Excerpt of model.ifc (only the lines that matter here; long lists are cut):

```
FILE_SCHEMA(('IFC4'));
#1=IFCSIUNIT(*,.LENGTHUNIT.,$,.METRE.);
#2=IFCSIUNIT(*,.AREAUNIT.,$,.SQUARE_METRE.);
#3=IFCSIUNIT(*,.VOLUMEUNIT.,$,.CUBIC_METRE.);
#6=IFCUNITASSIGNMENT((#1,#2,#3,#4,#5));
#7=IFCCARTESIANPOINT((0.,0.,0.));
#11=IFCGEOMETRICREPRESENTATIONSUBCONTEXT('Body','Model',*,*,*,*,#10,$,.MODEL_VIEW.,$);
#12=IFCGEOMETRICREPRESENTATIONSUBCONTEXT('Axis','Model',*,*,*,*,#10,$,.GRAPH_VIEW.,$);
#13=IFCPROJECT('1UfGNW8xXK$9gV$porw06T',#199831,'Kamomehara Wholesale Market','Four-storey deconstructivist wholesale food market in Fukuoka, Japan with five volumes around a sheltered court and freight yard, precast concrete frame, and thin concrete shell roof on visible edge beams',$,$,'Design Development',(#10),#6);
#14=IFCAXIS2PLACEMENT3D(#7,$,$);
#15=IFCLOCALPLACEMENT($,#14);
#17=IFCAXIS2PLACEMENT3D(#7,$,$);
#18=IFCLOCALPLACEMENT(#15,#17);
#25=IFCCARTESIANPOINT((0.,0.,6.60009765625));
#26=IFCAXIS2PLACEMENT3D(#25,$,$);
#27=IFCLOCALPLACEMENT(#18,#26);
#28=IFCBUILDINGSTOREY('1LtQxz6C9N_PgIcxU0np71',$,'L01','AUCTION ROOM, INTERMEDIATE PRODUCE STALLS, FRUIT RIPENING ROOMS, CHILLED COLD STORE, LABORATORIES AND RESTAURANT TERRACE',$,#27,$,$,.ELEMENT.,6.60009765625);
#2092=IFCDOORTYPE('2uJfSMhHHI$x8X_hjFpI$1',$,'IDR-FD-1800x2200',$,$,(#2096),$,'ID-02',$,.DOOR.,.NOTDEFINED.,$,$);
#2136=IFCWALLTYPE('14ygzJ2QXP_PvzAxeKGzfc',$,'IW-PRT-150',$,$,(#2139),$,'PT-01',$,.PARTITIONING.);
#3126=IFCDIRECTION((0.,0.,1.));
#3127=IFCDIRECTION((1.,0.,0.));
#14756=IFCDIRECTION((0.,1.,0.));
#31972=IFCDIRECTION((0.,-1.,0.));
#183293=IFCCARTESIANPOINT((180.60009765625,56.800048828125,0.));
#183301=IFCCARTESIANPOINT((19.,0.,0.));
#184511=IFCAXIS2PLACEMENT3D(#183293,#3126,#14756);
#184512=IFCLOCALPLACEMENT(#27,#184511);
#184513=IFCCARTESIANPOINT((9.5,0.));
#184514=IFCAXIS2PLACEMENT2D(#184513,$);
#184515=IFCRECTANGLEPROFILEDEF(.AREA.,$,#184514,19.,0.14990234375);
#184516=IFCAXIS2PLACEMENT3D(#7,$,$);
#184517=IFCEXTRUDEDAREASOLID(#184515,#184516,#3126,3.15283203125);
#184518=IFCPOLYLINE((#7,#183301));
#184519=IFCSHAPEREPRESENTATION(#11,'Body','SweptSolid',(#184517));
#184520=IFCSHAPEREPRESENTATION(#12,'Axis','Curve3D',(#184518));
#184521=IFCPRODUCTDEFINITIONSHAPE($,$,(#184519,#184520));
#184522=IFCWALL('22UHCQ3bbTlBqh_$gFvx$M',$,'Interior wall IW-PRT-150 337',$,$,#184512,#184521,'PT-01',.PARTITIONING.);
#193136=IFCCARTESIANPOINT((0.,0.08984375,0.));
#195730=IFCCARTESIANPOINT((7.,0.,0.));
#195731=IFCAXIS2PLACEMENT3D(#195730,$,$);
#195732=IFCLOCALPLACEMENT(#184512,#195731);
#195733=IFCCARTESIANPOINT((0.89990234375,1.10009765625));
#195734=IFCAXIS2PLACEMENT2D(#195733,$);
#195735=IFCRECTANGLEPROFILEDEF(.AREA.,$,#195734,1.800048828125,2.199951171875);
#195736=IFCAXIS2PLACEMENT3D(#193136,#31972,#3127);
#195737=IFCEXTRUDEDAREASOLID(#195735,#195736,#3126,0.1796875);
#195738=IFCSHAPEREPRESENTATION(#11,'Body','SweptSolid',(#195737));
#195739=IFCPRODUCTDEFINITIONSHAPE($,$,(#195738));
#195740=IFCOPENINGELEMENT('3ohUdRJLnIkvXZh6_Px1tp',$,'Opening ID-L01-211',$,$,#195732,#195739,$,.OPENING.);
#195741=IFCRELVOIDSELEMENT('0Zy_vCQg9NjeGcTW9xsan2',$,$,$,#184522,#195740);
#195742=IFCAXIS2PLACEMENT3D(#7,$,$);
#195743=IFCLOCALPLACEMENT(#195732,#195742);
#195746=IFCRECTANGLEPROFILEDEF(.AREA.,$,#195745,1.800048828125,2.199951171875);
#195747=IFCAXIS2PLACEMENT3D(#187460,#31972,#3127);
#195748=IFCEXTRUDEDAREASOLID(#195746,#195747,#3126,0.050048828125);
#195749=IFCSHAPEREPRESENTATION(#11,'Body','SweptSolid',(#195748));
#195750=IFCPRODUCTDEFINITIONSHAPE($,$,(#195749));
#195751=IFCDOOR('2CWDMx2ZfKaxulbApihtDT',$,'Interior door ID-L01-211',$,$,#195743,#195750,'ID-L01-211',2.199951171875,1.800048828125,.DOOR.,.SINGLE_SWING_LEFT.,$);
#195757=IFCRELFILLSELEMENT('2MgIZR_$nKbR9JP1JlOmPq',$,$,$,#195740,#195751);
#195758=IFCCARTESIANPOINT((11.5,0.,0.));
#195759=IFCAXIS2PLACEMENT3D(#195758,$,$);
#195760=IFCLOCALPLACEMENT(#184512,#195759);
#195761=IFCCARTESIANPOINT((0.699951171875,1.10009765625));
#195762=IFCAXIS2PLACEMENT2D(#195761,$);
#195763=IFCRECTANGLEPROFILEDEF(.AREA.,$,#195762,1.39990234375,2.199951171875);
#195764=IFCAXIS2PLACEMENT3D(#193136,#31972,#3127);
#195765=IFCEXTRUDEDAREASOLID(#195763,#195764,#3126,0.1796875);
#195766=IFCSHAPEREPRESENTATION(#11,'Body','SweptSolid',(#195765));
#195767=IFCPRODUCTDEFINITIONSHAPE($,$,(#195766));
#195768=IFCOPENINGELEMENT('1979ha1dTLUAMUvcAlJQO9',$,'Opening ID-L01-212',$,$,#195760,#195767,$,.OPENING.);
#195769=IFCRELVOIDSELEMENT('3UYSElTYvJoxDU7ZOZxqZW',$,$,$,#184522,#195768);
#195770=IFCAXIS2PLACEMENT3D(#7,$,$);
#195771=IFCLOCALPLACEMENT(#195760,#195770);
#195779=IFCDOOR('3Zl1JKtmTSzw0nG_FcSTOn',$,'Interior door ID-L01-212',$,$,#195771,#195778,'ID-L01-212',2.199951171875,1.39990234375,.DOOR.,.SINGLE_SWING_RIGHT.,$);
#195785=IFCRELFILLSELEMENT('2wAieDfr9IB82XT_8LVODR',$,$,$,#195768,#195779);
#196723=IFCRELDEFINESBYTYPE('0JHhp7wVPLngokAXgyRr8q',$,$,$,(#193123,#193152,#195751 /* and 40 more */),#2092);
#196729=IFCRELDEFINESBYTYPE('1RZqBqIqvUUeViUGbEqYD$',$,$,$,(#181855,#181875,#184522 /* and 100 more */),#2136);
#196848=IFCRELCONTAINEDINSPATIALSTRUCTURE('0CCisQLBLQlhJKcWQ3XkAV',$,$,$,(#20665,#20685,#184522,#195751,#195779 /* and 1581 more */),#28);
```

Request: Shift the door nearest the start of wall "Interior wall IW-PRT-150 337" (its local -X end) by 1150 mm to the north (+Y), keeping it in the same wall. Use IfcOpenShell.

```python
import ifcopenshell
import ifcopenshell.api.geometry
import ifcopenshell.util.placement
import ifcopenshell.util.unit

model = ifcopenshell.open("model.ifc")
unit_scale = ifcopenshell.util.unit.calculate_unit_scale(model)

door = model.by_guid("2CWDMx2ZfKaxulbApihtDT")
opening = door.FillsVoids[0].RelatingOpeningElement
wall = opening.VoidsElements[0].RelatingBuildingElement

wall_matrix = ifcopenshell.util.placement.get_local_placement(wall.ObjectPlacement)
shift = wall_matrix[:3, 0] * 1.15 / unit_scale
before = ifcopenshell.util.placement.get_local_placement(door.ObjectPlacement)[:3, 3].copy()

# The door is placed relative to its opening, so it follows when the opening moves.
matrix = ifcopenshell.util.placement.get_local_placement(opening.ObjectPlacement)
matrix[:3, 3] += shift
ifcopenshell.api.geometry.edit_object_placement(
    model, product=opening, matrix=matrix, is_si=False, should_transform_children=True
)

after = ifcopenshell.util.placement.get_local_placement(door.ObjectPlacement)[:3, 3]
print("door moved by", (after - before).round(3) + 0.0)

model.write("model_v2.ifc")
```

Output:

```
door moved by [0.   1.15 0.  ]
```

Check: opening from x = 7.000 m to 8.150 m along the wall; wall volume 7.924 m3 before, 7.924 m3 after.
